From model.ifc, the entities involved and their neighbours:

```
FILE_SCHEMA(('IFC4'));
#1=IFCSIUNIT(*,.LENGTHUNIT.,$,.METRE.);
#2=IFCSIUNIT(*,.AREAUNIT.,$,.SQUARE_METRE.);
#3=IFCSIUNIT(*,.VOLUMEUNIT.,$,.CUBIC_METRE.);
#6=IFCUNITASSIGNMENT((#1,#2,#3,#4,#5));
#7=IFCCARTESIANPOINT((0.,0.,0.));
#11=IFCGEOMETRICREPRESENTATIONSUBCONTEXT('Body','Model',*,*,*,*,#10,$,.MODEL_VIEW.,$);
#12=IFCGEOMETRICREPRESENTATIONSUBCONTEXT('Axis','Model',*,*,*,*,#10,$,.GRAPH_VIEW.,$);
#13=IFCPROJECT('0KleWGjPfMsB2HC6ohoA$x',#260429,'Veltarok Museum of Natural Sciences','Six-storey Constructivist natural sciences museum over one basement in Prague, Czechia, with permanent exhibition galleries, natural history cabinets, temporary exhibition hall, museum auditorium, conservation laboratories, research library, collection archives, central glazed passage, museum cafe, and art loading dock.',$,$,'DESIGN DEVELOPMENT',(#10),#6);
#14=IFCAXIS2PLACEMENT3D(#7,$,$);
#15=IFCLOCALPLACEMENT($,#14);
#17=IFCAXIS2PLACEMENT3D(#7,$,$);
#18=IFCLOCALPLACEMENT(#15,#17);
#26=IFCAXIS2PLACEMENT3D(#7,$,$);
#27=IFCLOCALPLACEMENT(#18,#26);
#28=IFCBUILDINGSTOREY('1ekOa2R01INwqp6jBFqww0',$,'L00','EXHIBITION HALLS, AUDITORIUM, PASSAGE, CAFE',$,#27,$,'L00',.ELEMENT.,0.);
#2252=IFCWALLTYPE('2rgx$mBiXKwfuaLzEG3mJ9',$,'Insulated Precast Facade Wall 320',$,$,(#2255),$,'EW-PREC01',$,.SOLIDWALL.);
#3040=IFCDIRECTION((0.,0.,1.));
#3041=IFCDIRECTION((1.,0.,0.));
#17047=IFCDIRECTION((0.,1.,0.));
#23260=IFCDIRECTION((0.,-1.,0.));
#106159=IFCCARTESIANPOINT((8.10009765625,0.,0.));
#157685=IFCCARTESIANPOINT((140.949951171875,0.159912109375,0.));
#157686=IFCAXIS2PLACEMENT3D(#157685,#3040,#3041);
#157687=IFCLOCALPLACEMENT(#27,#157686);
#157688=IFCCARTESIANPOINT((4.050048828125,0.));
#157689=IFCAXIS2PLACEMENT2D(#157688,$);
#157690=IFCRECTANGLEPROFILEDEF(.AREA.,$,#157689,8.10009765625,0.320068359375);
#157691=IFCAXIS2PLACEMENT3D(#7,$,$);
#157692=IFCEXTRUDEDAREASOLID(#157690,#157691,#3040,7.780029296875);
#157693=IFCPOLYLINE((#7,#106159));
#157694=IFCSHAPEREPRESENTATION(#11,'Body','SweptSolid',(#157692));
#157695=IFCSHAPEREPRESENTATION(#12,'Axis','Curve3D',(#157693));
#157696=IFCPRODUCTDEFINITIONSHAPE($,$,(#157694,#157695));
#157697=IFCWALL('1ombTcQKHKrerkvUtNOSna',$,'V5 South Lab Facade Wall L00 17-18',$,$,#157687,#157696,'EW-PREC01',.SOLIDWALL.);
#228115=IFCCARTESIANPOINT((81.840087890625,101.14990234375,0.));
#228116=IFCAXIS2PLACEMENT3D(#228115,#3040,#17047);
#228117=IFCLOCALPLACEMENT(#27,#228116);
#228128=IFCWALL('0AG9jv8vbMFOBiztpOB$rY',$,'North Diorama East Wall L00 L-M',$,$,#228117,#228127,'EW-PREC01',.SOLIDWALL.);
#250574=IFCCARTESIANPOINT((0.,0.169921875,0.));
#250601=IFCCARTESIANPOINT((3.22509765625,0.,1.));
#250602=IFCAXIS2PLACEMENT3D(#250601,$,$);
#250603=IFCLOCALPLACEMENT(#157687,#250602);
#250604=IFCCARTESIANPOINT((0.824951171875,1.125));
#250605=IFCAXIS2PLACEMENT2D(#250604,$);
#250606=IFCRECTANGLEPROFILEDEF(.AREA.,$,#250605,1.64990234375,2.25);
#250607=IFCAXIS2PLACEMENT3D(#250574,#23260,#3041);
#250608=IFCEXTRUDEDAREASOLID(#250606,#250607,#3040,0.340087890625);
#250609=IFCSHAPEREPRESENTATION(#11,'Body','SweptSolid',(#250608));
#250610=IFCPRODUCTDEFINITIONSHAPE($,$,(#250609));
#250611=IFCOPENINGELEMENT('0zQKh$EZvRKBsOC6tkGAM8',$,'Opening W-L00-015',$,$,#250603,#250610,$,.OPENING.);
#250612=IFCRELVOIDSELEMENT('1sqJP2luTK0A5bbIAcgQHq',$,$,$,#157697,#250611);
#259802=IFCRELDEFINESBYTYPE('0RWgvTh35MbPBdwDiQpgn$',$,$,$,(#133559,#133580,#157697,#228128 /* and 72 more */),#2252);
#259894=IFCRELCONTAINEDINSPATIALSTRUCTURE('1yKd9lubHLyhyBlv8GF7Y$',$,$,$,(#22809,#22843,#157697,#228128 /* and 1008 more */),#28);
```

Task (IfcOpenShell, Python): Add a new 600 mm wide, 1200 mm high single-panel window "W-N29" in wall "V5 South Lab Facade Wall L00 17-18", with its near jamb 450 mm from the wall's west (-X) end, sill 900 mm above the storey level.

```python
import numpy as np
import ifcopenshell
import ifcopenshell.api.feature
import ifcopenshell.api.geometry
import ifcopenshell.api.root
import ifcopenshell.api.spatial
import ifcopenshell.geom
import ifcopenshell.util.element
import ifcopenshell.util.placement
import ifcopenshell.util.representation
import ifcopenshell.util.shape
import ifcopenshell.util.unit

model = ifcopenshell.open("model.ifc")
unit_scale = ifcopenshell.util.unit.calculate_unit_scale(model)
settings = ifcopenshell.geom.settings()


def volume(element):
    """Net volume in cubic metres, openings subtracted."""
    shape = ifcopenshell.geom.create_shape(settings, element)
    return ifcopenshell.util.shape.get_volume(shape.geometry)


wall = model.by_guid("1ombTcQKHKrerkvUtNOSna")
storey = ifcopenshell.util.element.get_container(wall, ifc_class="IfcBuildingStorey")
context = ifcopenshell.util.representation.get_context(model, "Model", "Body", "MODEL_VIEW")
before = volume(wall)

width, height, from_end, sill = 0.6, 1.2, 0.45, 0.9  # metres

# The wall runs along its own X axis, and the end named is its -X end.
wall_shape = ifcopenshell.geom.create_shape(settings, wall)
x, y, z = ifcopenshell.util.shape.get_vertices(wall_shape.geometry).T
start = x.min() + from_end
face, thickness = float(y.min()), float(y.max() - y.min())
wall_matrix = ifcopenshell.util.placement.get_local_placement(wall.ObjectPlacement)
level = ifcopenshell.util.placement.get_local_placement(storey.ObjectPlacement)[2, 3]


def in_wall(x, y):
    """Placement at x, y metres in the wall's axes, at sill height."""
    matrix = wall_matrix.copy()
    matrix[:, 3] = wall_matrix @ np.array([x / unit_scale, y / unit_scale, 0.0, 1.0])
    matrix[2, 3] = level + sill / unit_scale
    return matrix


# Opening: a box that overshoots both wall faces by 50 mm.
opening = ifcopenshell.api.root.create_entity(model, ifc_class="IfcOpeningElement", predefined_type="OPENING")
box = ifcopenshell.api.geometry.add_wall_representation(
    model, context=context, length=width, height=height, thickness=thickness + 0.1
)
ifcopenshell.api.geometry.assign_representation(model, product=opening, representation=box)
ifcopenshell.api.geometry.edit_object_placement(model, product=opening, matrix=in_wall(start, face - 0.05), is_si=False)
ifcopenshell.api.feature.add_feature(model, feature=opening, element=wall)

window = ifcopenshell.api.root.create_entity(model, ifc_class="IfcWindow", name="W-N29", predefined_type="WINDOW")
window.OverallWidth, window.OverallHeight = width / unit_scale, height / unit_scale
window.PartitioningType = "SINGLE_PANEL"
body = ifcopenshell.api.geometry.add_window_representation(
    model,
    context=context,
    overall_width=window.OverallWidth,
    overall_height=window.OverallHeight,
    partition_type="SINGLE_PANEL",
)
ifcopenshell.api.geometry.assign_representation(model, product=window, representation=body)
ifcopenshell.api.spatial.assign_container(model, products=[window], relating_structure=storey)
ifcopenshell.api.feature.add_filling(model, opening=opening, element=window)

# Centre the window in the wall's thickness.
ifcopenshell.api.geometry.edit_object_placement(model, product=window, matrix=in_wall(start, face), is_si=False)
window_shape = ifcopenshell.geom.create_shape(settings, window)
depth = ifcopenshell.util.shape.get_vertices(window_shape.geometry)[:, 1]
offset = face + thickness / 2 - (depth.min() + depth.max()) / 2
ifcopenshell.api.geometry.edit_object_placement(model, product=window, matrix=in_wall(start, offset), is_si=False)

after = volume(wall)

print(f"wall volume {before:.3f} -> {after:.3f} m3")

model.write("model_updated.ifc")
```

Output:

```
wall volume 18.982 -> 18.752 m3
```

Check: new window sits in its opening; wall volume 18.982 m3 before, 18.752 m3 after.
